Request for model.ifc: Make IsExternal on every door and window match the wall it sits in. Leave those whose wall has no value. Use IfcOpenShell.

First a look at what the model holds.

```python
import ifcopenshell
import ifcopenshell.util.element

model = ifcopenshell.open("model.ifc")
print(model.schema)
seen = {}
for e in model.by_type("IfcDoor") + model.by_type("IfcWindow"):
    if not e.FillsVoids:
        continue
    host = e.FillsVoids[0].RelatingOpeningElement.VoidsElements[0].RelatingBuildingElement
    own = ifcopenshell.util.element.get_pset(e, f"Pset_{e.is_a()[3:].removesuffix('StandardCase')}Common", "IsExternal")
    wall = ifcopenshell.util.element.get_pset(host, "Pset_WallCommon", "IsExternal")
    seen[e.is_a(), own, wall] = seen.get((e.is_a(), own, wall), 0) + 1
for (cls, own, wall), count in sorted(seen.items(), key=str):
    print(count, cls, "IsExternal:", own, "| host wall:", wall)
```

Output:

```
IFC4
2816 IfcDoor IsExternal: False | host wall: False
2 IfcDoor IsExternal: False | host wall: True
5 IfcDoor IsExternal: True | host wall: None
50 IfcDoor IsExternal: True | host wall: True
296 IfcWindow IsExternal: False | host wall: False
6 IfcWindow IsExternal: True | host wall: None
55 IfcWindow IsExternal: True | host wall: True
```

```python
import ifcopenshell
import ifcopenshell.api.pset
import ifcopenshell.util.element

model = ifcopenshell.open("model.ifc")

count = 0
for ifc_class, pset_name in (("IfcDoor", "Pset_DoorCommon"), ("IfcWindow", "Pset_WindowCommon")):
    for e in model.by_type(ifc_class):
        if not e.FillsVoids:
            continue
        host = e.FillsVoids[0].RelatingOpeningElement.VoidsElements[0].RelatingBuildingElement
        external = ifcopenshell.util.element.get_pset(host, "Pset_WallCommon", "IsExternal")
        if external is None or ifcopenshell.util.element.get_pset(e, pset_name, "IsExternal") == external:
            continue
        found = ifcopenshell.util.element.get_pset(e, pset_name, should_inherit=False)
        if found:
            pset = model.by_id(found["id"])
            if len(ifcopenshell.util.element.get_elements_by_pset(pset)) > 1:
                pset = ifcopenshell.api.pset.unshare_pset(model, products=[e], pset=pset)[0]
        else:
            pset = ifcopenshell.api.pset.add_pset(model, product=e, name=pset_name)
        ifcopenshell.api.pset.edit_pset(model, pset=pset, properties={"IsExternal": external})
        count += 1

print(count, "updated")

model.write("model_v2.ifc")
```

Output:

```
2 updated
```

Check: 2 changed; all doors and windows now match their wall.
